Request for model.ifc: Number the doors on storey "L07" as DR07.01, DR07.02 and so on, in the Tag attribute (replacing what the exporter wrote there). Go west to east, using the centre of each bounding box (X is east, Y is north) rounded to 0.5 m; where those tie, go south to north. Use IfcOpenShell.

First a look at what the model holds.

```python
import ifcopenshell
import ifcopenshell.util.element
import ifcopenshell.util.placement

model = ifcopenshell.open("model.ifc")
print(model.schema)
storey = next(s for s in model.by_type("IfcBuildingStorey") if s.Name == "L07")
doors = [e for e in ifcopenshell.util.element.get_decomposition(storey) if e.is_a("IfcDoor")]
for e in sorted(doors, key=lambda e: e.id()):
    origin = ifcopenshell.util.placement.get_local_placement(e.ObjectPlacement)[:3, 3]
    print(e.id(), e.Tag, e.Name, origin.round(2) + 0.0, sep=" | ")
```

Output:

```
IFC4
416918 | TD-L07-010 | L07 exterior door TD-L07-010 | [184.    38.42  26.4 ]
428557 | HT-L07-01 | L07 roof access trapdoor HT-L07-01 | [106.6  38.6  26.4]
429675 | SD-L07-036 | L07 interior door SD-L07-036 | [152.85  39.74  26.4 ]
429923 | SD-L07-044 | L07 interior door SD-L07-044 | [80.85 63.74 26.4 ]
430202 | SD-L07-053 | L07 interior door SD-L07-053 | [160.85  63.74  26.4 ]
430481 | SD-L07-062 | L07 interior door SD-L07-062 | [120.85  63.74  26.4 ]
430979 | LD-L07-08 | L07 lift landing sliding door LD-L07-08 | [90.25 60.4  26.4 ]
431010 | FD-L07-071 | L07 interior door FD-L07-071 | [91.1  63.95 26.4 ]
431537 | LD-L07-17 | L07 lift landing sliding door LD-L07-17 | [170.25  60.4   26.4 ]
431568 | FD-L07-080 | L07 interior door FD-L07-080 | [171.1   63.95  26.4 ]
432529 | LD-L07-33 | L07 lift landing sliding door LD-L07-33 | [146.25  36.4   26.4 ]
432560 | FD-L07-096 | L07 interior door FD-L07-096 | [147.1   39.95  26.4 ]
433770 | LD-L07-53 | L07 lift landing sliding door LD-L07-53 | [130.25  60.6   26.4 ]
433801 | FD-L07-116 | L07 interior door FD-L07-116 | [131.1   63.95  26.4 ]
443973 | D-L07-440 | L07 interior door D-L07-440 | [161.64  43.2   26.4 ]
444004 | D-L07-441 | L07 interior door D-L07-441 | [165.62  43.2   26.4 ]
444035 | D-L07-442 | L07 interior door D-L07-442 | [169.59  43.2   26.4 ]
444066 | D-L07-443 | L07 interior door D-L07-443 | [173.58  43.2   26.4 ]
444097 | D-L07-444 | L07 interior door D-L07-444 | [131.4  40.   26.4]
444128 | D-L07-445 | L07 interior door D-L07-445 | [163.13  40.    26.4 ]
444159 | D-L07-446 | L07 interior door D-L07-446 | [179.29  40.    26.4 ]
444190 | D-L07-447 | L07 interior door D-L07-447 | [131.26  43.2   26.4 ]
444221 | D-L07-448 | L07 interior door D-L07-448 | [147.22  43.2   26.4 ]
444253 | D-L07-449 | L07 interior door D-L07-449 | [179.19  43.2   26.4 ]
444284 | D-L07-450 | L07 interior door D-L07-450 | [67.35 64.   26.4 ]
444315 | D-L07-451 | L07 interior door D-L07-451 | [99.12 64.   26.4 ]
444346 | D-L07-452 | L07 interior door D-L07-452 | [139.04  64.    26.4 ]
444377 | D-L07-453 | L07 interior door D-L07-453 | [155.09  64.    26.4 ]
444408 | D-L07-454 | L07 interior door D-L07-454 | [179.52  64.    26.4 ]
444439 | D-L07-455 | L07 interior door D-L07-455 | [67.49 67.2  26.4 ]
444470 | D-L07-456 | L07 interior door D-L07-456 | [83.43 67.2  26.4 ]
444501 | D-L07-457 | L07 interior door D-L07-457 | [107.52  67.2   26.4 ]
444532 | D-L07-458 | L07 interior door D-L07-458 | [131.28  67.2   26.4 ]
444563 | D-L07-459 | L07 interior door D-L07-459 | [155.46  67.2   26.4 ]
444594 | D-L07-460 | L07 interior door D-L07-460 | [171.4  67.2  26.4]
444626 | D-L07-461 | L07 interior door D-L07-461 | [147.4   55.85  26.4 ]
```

```python
import ifcopenshell
import ifcopenshell.geom
import ifcopenshell.util.element
import ifcopenshell.util.shape

model = ifcopenshell.open("model.ifc")
settings = ifcopenshell.geom.settings()
settings.set("use-world-coords", True)


def centre(element):
    shape = ifcopenshell.geom.create_shape(settings, element)
    return ifcopenshell.util.shape.get_bbox_centroid(shape.geometry)


storey = next(s for s in model.by_type("IfcBuildingStorey") if s.Name == "L07")
doors = [e for e in ifcopenshell.util.element.get_decomposition(storey) if e.is_a("IfcDoor")]

# Insertion points can sit at a corner or the storey origin, so sort by the geometry (in metres).
centres = {e: centre(e) for e in doors}
doors.sort(key=lambda e: (round(centres[e][0] / 0.5), centres[e][1]))

for i, e in enumerate(doors, start=1):
    number = f"DR07.{i:02d}"
    e.Tag = number
    print(e.id(), number)

model.write("model_v2.ifc")
```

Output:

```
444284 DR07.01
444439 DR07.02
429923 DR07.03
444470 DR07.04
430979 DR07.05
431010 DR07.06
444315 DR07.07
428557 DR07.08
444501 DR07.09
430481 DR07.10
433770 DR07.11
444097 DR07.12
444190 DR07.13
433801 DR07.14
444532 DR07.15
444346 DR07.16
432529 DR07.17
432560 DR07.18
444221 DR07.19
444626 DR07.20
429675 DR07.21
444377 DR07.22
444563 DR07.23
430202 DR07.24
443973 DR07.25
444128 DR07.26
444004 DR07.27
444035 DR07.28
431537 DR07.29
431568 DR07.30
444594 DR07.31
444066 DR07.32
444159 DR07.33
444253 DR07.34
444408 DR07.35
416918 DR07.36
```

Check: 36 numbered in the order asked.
